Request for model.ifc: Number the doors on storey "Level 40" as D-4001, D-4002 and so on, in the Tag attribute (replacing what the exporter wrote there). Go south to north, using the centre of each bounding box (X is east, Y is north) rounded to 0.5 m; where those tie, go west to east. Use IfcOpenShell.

First a look at what the model holds.

```python
import ifcopenshell
import ifcopenshell.util.element
import ifcopenshell.util.placement

model = ifcopenshell.open("model.ifc")
print(model.schema)
storey = next(s for s in model.by_type("IfcBuildingStorey") if s.Name == "Level 40")
doors = [e for e in ifcopenshell.util.element.get_decomposition(storey) if e.is_a("IfcDoor")]
for e in sorted(doors, key=lambda e: e.id()):
    origin = ifcopenshell.util.placement.get_local_placement(e.ObjectPlacement)[:3, 3]
    print(e.id(), e.Tag, e.Name, origin.round(2) + 0.0, sep=" | ")
```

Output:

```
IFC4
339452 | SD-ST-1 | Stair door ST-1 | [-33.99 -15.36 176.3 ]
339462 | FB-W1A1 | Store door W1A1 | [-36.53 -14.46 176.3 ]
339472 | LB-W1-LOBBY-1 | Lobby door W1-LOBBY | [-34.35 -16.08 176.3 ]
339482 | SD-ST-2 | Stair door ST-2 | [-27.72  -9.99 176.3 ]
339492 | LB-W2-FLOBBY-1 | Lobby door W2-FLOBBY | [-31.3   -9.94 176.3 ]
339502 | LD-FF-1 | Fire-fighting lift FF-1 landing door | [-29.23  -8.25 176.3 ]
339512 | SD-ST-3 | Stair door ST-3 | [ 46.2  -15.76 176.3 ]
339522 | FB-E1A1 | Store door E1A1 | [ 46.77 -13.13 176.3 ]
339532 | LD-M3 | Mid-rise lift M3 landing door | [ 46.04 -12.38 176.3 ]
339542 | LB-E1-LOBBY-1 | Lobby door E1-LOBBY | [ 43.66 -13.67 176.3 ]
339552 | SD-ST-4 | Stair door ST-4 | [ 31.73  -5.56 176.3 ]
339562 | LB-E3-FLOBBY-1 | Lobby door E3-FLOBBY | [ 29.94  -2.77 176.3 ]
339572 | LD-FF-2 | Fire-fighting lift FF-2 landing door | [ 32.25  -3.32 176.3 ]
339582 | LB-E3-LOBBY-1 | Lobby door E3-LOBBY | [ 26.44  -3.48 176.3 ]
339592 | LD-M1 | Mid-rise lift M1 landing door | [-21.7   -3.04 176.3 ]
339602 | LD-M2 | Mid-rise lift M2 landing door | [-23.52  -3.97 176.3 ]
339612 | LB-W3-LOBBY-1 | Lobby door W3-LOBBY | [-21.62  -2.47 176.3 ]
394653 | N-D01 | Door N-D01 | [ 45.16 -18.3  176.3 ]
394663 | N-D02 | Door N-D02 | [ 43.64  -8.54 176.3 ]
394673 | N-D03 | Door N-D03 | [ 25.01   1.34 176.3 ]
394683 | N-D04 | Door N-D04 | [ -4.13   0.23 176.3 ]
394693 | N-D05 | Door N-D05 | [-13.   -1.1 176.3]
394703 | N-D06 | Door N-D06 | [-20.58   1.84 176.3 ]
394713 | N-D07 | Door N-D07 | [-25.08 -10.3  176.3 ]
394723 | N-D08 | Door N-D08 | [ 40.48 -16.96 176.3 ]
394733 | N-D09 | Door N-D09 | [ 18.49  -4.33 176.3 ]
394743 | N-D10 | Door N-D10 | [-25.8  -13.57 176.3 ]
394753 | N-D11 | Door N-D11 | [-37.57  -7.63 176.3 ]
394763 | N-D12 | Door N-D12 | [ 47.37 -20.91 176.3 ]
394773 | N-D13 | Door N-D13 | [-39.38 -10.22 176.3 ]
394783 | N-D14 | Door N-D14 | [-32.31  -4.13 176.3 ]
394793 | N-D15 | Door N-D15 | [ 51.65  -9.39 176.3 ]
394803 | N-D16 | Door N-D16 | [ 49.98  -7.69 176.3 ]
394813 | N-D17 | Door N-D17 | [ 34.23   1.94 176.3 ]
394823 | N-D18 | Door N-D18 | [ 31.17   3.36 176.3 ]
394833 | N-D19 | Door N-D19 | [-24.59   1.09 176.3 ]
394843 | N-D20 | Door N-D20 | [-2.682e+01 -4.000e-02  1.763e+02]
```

```python
import ifcopenshell
import ifcopenshell.geom
import ifcopenshell.util.element
import ifcopenshell.util.shape

model = ifcopenshell.open("model.ifc")
settings = ifcopenshell.geom.settings()
settings.set("use-world-coords", True)


def centre(element):
    shape = ifcopenshell.geom.create_shape(settings, element)
    return ifcopenshell.util.shape.get_bbox_centroid(shape.geometry)


storey = next(s for s in model.by_type("IfcBuildingStorey") if s.Name == "Level 40")
doors = [e for e in ifcopenshell.util.element.get_decomposition(storey) if e.is_a("IfcDoor")]

# Insertion points can sit at a corner or the storey origin, so sort by the geometry (in metres).
centres = {e: centre(e) for e in doors}
doors.sort(key=lambda e: (round(centres[e][1] / 0.5), centres[e][0]))

for i, e in enumerate(doors, start=1):
    number = f"D-40{i:02d}"
    e.Tag = number
    print(e.id(), number)

model.write("model_rev.ifc")
```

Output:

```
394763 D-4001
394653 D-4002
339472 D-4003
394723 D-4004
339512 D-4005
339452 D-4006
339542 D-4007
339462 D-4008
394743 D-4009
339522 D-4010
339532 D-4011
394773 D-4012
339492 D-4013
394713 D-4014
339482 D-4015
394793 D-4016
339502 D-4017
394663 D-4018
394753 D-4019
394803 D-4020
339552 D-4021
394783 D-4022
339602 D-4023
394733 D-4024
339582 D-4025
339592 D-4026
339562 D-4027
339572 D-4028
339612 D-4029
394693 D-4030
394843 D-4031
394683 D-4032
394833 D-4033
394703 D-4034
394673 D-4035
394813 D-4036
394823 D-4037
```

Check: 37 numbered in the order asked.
